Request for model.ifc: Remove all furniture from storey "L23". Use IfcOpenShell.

First a look at what the model holds.

```python
import ifcopenshell
import ifcopenshell.util.element

model = ifcopenshell.open("model.ifc")
print(model.schema)
storey = next(s for s in model.by_type("IfcBuildingStorey") if s.Name == "L23")
furniture = [e for e in ifcopenshell.util.element.get_decomposition(storey) if e.is_a("IfcFurnishingElement")]
seen = {}
for e in furniture:
    element_type = ifcopenshell.util.element.get_type(e)
    name = element_type.Name if element_type not in (None, e) else None
    seen[name] = seen.get(name, 0) + 1
for name, count in sorted(seen.items(), key=str):
    print(count, "x", name)
```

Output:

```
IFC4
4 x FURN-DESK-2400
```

```python
import ifcopenshell
import ifcopenshell.api.root
import ifcopenshell.util.element

model = ifcopenshell.open("model.ifc")

storey = next(s for s in model.by_type("IfcBuildingStorey") if s.Name == "L23")
furniture = [e for e in ifcopenshell.util.element.get_decomposition(storey) if e.is_a("IfcFurnishingElement")]

for e in furniture:
    ifcopenshell.api.root.remove_product(model, product=e)
print(len(furniture), "removed")

model.write("model_updated.ifc")
```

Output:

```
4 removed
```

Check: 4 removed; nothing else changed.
